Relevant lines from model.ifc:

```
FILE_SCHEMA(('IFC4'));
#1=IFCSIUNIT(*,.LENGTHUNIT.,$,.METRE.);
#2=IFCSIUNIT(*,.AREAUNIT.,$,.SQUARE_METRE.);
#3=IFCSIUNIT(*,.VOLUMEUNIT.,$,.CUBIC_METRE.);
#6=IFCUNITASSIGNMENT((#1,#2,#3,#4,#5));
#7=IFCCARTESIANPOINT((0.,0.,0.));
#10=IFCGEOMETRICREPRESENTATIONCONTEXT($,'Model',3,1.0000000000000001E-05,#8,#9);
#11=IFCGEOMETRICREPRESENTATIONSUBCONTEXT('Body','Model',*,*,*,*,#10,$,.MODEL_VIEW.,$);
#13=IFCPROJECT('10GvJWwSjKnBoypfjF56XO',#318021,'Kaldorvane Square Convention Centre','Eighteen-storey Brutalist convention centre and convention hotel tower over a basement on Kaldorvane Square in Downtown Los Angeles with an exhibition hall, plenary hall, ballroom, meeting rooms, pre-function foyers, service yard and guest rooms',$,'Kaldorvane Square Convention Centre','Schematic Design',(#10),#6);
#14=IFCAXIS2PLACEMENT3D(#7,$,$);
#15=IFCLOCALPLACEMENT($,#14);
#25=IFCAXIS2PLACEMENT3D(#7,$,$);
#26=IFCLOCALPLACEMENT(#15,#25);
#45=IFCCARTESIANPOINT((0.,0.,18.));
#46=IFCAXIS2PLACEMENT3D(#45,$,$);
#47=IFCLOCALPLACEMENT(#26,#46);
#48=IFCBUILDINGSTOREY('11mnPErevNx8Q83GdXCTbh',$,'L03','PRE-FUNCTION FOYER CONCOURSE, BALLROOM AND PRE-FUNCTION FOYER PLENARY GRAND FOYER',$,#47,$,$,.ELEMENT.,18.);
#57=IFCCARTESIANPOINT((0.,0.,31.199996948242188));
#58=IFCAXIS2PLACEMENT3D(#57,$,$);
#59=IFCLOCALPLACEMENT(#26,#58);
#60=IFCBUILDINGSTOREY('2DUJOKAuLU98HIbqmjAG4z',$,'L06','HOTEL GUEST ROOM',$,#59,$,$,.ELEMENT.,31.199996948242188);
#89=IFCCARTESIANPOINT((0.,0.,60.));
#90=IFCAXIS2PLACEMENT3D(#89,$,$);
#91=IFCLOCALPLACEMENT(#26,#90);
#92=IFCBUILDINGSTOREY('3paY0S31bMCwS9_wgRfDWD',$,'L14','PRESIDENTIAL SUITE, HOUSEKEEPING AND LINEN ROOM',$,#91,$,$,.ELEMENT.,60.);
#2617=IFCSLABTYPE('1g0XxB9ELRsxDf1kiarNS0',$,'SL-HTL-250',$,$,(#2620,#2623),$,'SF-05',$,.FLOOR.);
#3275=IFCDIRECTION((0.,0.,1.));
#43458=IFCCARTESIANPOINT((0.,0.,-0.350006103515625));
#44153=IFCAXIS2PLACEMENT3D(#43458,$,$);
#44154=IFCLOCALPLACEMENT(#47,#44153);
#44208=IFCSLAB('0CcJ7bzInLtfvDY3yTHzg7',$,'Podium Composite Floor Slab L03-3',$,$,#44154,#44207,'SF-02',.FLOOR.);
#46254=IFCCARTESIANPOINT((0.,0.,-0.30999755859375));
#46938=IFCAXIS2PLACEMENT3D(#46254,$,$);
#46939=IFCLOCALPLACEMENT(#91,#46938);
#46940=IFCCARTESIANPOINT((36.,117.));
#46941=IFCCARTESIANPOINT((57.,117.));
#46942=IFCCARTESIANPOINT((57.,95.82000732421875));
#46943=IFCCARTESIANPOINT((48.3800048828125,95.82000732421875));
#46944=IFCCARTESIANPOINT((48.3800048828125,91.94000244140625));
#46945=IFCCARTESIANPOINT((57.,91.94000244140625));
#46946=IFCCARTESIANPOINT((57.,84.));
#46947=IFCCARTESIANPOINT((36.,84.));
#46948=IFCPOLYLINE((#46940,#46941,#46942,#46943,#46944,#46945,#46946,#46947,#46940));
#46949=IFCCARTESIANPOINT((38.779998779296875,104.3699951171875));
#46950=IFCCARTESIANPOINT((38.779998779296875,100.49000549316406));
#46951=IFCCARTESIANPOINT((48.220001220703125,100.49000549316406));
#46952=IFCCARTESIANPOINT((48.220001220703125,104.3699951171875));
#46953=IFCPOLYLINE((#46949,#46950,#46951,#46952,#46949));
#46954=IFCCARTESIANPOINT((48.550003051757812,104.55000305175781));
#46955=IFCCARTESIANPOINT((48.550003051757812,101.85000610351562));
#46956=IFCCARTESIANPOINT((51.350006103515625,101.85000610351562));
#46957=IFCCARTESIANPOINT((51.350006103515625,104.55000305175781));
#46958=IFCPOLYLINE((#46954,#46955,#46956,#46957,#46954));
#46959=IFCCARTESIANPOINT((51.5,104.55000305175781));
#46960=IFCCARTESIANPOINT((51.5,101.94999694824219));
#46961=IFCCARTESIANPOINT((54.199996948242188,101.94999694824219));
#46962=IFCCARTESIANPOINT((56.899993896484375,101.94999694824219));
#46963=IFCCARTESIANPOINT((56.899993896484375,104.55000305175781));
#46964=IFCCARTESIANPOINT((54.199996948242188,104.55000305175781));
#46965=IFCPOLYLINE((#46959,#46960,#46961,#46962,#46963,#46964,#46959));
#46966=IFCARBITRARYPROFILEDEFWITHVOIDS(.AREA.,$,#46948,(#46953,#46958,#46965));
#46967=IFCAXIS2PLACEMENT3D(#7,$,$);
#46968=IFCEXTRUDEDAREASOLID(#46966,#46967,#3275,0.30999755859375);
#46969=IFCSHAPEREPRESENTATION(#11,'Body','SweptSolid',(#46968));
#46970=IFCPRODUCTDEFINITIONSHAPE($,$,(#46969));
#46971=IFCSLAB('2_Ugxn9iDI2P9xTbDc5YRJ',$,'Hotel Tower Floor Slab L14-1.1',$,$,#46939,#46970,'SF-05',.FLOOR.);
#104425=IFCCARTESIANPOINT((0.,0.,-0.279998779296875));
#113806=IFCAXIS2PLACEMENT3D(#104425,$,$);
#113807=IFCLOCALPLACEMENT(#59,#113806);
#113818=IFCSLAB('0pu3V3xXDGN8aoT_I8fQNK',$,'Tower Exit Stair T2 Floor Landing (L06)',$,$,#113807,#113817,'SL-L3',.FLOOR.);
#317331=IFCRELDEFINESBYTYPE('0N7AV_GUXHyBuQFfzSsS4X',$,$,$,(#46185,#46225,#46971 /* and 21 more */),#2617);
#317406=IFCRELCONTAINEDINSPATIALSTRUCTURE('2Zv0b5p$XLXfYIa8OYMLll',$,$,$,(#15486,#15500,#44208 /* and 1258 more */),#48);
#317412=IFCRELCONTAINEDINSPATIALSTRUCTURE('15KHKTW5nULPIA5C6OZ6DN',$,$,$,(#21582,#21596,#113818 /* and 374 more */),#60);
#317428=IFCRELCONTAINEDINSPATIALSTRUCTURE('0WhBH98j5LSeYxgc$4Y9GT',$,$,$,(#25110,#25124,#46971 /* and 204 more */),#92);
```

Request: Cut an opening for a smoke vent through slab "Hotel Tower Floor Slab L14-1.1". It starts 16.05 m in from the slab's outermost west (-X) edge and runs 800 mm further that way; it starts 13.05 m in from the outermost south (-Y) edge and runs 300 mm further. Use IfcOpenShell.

```python
import numpy as np
import ifcopenshell
import ifcopenshell.api.feature
import ifcopenshell.api.geometry
import ifcopenshell.api.root
import ifcopenshell.geom
import ifcopenshell.util.placement
import ifcopenshell.util.representation
import ifcopenshell.util.shape
import ifcopenshell.util.unit

model = ifcopenshell.open("model.ifc")
unit_scale = ifcopenshell.util.unit.calculate_unit_scale(model)
settings = ifcopenshell.geom.settings()


def volume(element):
    """Net volume in cubic metres, openings subtracted."""
    shape = ifcopenshell.geom.create_shape(settings, element)
    return ifcopenshell.util.shape.get_volume(shape.geometry)


slab = model.by_id(46971)
before = volume(slab)

# Extent in the slab's own axes, in metres. The edges named are its -X and -Y sides.
slab_shape = ifcopenshell.geom.create_shape(settings, slab)
vertices = ifcopenshell.util.shape.get_vertices(slab_shape.geometry)
x_min, y_min, bottom = vertices.min(axis=0)
top = vertices[:, 2].max()

opening = ifcopenshell.api.root.create_entity(model, ifc_class="IfcOpeningElement", name="Smoke vent opening", predefined_type="OPENING")
context = ifcopenshell.util.representation.get_context(model, "Model", "Body", "MODEL_VIEW")
width, depth = 0.8, 0.3
outline = [(0.0, 0.0), (width, 0.0), (width, depth), (0.0, depth), (0.0, 0.0)]
# Overshoot both faces by 50 mm so the cut is clean.
shape = ifcopenshell.api.geometry.add_slab_representation(
    model, context=context, depth=top - bottom + 0.1, polyline=outline
)
ifcopenshell.api.geometry.assign_representation(model, product=opening, representation=shape)

matrix = ifcopenshell.util.placement.get_local_placement(slab.ObjectPlacement)
matrix[:, 3] = matrix @ np.append(np.array([x_min + 16.05, y_min + 13.05, bottom - 0.05]) / unit_scale, 1.0)
ifcopenshell.api.geometry.edit_object_placement(model, product=opening, matrix=matrix, is_si=False)
ifcopenshell.api.feature.add_feature(model, feature=opening, element=slab)

after = volume(slab)

print(f"slab volume {before:.3f} -> {after:.3f} m3")

model.write("model_updated.ifc")
```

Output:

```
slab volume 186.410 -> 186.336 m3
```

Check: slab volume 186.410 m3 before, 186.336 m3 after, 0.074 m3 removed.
